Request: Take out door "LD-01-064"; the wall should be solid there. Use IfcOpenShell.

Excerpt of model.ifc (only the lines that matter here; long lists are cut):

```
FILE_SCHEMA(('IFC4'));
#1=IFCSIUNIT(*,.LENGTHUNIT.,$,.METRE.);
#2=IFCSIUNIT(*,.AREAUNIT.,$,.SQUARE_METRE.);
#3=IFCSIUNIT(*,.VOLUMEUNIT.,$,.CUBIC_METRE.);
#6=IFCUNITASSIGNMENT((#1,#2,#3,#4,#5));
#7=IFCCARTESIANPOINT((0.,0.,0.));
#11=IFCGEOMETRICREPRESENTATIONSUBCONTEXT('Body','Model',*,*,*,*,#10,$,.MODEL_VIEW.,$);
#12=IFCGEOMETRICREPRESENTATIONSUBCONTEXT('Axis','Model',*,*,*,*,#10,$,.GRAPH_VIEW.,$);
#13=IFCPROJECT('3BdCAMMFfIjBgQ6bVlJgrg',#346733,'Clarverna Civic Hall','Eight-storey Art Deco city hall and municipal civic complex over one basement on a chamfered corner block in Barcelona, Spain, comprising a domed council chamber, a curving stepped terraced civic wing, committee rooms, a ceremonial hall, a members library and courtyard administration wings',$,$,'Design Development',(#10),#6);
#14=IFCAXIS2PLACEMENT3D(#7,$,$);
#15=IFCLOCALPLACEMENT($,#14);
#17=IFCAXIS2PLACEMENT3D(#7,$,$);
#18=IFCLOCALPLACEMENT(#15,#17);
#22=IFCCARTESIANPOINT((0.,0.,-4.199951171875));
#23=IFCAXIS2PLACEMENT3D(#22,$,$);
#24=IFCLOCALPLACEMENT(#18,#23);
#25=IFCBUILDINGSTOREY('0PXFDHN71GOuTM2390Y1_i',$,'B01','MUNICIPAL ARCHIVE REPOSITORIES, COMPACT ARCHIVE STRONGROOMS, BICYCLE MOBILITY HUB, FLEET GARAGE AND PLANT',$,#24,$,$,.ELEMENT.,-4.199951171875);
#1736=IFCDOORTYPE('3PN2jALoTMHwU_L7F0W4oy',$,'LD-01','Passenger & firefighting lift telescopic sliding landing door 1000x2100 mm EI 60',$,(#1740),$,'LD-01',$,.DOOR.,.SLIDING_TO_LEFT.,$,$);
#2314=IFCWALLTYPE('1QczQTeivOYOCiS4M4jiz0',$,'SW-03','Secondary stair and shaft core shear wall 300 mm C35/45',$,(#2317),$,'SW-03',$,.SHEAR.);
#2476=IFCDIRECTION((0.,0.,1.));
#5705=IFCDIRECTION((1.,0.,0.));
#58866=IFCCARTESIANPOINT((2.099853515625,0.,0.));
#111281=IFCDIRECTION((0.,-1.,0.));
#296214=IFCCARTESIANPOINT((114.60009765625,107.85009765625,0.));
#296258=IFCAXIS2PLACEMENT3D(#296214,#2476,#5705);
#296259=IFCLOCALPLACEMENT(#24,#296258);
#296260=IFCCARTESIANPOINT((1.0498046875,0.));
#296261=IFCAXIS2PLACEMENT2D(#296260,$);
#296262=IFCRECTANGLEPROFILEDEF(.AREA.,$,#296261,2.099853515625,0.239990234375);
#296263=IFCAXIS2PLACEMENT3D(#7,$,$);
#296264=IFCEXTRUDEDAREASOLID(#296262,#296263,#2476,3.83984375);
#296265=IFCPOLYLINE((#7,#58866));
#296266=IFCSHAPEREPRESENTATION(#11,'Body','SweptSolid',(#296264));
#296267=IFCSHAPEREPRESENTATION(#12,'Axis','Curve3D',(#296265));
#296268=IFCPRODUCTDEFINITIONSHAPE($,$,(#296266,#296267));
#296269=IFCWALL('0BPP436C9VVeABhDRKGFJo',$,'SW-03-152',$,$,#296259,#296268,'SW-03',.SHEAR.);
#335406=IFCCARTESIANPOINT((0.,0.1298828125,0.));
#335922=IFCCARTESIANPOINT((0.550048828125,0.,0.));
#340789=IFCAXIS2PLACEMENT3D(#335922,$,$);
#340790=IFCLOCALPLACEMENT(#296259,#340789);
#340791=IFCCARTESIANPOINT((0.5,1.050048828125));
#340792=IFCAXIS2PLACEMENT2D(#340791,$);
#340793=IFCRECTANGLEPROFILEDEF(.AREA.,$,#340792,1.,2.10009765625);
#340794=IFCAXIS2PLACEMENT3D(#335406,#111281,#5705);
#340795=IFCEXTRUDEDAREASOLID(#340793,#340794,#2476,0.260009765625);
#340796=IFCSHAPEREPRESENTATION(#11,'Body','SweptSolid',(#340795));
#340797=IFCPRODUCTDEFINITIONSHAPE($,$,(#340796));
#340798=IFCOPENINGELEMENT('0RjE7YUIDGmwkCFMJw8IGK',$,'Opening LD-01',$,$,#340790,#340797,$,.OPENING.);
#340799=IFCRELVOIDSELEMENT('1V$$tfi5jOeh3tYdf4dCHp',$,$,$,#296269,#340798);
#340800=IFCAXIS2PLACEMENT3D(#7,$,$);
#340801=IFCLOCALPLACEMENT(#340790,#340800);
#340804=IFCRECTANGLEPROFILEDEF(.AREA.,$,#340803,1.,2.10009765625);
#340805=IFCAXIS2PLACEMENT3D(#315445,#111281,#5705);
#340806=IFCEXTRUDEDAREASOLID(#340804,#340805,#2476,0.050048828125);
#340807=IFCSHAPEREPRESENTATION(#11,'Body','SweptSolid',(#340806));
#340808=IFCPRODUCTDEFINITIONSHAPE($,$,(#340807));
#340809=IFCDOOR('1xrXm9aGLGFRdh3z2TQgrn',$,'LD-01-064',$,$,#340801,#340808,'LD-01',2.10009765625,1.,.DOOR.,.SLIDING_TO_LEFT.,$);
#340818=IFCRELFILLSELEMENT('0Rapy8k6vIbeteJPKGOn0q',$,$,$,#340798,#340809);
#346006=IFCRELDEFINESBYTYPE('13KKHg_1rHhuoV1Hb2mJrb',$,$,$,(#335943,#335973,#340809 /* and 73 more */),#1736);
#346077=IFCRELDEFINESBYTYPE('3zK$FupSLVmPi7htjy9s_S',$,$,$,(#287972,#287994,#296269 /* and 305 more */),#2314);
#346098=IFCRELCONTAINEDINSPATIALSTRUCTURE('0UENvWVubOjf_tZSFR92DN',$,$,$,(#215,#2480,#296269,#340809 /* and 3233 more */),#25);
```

```python
import ifcopenshell
import ifcopenshell.api.feature
import ifcopenshell.api.root
import ifcopenshell.geom
import ifcopenshell.util.shape

model = ifcopenshell.open("model.ifc")
settings = ifcopenshell.geom.settings()


def volume(element):
    """Net volume in cubic metres, openings subtracted."""
    shape = ifcopenshell.geom.create_shape(settings, element)
    return ifcopenshell.util.shape.get_volume(shape.geometry)


door = model.by_guid("1xrXm9aGLGFRdh3z2TQgrn")
opening = door.FillsVoids[0].RelatingOpeningElement
wall = opening.VoidsElements[0].RelatingBuildingElement
before = volume(wall)

ifcopenshell.api.root.remove_product(model, product=door)
ifcopenshell.api.feature.remove_feature(model, feature=opening)

after = volume(wall)

print(f"wall volume {before:.3f} -> {after:.3f} m3")

model.write("model_edited.ifc")
```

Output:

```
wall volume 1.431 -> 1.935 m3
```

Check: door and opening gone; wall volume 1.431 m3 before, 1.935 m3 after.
